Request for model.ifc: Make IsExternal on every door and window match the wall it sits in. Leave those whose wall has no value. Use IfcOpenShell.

First a look at what the model holds.

```python
import ifcopenshell
import ifcopenshell.util.element

model = ifcopenshell.open("model.ifc")
print(model.schema)
seen = {}
for e in model.by_type("IfcDoor") + model.by_type("IfcWindow"):
    if not e.FillsVoids:
        continue
    host = e.FillsVoids[0].RelatingOpeningElement.VoidsElements[0].RelatingBuildingElement
    own = ifcopenshell.util.element.get_pset(e, f"Pset_{e.is_a()[3:].removesuffix('StandardCase')}Common", "IsExternal")
    wall = ifcopenshell.util.element.get_pset(host, "Pset_WallCommon", "IsExternal")
    seen[e.is_a(), own, wall] = seen.get((e.is_a(), own, wall), 0) + 1
for (cls, own, wall), count in sorted(seen.items(), key=str):
    print(count, cls, "IsExternal:", own, "| host wall:", wall)
```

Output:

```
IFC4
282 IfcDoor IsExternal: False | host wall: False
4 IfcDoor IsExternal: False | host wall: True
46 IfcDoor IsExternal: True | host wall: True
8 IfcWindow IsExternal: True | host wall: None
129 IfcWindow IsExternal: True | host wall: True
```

```python
import ifcopenshell
import ifcopenshell.api.pset
import ifcopenshell.util.element

model = ifcopenshell.open("model.ifc")

count = 0
for ifc_class, pset_name in (("IfcDoor", "Pset_DoorCommon"), ("IfcWindow", "Pset_WindowCommon")):
    for e in model.by_type(ifc_class):
        if not e.FillsVoids:
            continue
        host = e.FillsVoids[0].RelatingOpeningElement.VoidsElements[0].RelatingBuildingElement
        external = ifcopenshell.util.element.get_pset(host, "Pset_WallCommon", "IsExternal")
        if external is None or ifcopenshell.util.element.get_pset(e, pset_name, "IsExternal") == external:
            continue
        pset = ifcopenshell.api.pset.add_pset(model, product=e, name=pset_name)
        ifcopenshell.api.pset.edit_pset(model, pset=pset, properties={"IsExternal": external})
        count += 1

print(count, "updated")

model.write("model_edited.ifc")
```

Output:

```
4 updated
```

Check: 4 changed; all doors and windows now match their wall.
